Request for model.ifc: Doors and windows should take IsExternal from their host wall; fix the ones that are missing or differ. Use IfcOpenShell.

First a look at what the model holds.

```python
import ifcopenshell
import ifcopenshell.util.element

model = ifcopenshell.open("model.ifc")
print(model.schema)
seen = {}
for e in model.by_type("IfcDoor") + model.by_type("IfcWindow"):
    if not e.FillsVoids:
        continue
    host = e.FillsVoids[0].RelatingOpeningElement.VoidsElements[0].RelatingBuildingElement
    own = ifcopenshell.util.element.get_pset(e, f"Pset_{e.is_a()[3:].removesuffix('StandardCase')}Common", "IsExternal")
    wall = ifcopenshell.util.element.get_pset(host, "Pset_WallCommon", "IsExternal")
    seen[e.is_a(), own, wall] = seen.get((e.is_a(), own, wall), 0) + 1
for (cls, own, wall), count in sorted(seen.items(), key=str):
    print(count, cls, "IsExternal:", own, "| host wall:", wall)
```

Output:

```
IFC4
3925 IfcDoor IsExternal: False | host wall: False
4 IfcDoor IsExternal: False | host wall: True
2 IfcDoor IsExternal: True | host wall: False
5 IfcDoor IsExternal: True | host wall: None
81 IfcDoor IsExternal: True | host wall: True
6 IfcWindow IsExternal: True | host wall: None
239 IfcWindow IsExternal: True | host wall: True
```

```python
import ifcopenshell
import ifcopenshell.api.pset
import ifcopenshell.util.element

model = ifcopenshell.open("model.ifc")

count = 0
for ifc_class, pset_name in (("IfcDoor", "Pset_DoorCommon"), ("IfcWindow", "Pset_WindowCommon")):
    for e in model.by_type(ifc_class):
        if not e.FillsVoids:
            continue
        host = e.FillsVoids[0].RelatingOpeningElement.VoidsElements[0].RelatingBuildingElement
        external = ifcopenshell.util.element.get_pset(host, "Pset_WallCommon", "IsExternal")
        if external is None or ifcopenshell.util.element.get_pset(e, pset_name, "IsExternal") == external:
            continue
        pset = ifcopenshell.api.pset.add_pset(model, product=e, name=pset_name)
        ifcopenshell.api.pset.edit_pset(model, pset=pset, properties={"IsExternal": external})
        count += 1

print(count, "updated")

model.write("model_edited.ifc")
```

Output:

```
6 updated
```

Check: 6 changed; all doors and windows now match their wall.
